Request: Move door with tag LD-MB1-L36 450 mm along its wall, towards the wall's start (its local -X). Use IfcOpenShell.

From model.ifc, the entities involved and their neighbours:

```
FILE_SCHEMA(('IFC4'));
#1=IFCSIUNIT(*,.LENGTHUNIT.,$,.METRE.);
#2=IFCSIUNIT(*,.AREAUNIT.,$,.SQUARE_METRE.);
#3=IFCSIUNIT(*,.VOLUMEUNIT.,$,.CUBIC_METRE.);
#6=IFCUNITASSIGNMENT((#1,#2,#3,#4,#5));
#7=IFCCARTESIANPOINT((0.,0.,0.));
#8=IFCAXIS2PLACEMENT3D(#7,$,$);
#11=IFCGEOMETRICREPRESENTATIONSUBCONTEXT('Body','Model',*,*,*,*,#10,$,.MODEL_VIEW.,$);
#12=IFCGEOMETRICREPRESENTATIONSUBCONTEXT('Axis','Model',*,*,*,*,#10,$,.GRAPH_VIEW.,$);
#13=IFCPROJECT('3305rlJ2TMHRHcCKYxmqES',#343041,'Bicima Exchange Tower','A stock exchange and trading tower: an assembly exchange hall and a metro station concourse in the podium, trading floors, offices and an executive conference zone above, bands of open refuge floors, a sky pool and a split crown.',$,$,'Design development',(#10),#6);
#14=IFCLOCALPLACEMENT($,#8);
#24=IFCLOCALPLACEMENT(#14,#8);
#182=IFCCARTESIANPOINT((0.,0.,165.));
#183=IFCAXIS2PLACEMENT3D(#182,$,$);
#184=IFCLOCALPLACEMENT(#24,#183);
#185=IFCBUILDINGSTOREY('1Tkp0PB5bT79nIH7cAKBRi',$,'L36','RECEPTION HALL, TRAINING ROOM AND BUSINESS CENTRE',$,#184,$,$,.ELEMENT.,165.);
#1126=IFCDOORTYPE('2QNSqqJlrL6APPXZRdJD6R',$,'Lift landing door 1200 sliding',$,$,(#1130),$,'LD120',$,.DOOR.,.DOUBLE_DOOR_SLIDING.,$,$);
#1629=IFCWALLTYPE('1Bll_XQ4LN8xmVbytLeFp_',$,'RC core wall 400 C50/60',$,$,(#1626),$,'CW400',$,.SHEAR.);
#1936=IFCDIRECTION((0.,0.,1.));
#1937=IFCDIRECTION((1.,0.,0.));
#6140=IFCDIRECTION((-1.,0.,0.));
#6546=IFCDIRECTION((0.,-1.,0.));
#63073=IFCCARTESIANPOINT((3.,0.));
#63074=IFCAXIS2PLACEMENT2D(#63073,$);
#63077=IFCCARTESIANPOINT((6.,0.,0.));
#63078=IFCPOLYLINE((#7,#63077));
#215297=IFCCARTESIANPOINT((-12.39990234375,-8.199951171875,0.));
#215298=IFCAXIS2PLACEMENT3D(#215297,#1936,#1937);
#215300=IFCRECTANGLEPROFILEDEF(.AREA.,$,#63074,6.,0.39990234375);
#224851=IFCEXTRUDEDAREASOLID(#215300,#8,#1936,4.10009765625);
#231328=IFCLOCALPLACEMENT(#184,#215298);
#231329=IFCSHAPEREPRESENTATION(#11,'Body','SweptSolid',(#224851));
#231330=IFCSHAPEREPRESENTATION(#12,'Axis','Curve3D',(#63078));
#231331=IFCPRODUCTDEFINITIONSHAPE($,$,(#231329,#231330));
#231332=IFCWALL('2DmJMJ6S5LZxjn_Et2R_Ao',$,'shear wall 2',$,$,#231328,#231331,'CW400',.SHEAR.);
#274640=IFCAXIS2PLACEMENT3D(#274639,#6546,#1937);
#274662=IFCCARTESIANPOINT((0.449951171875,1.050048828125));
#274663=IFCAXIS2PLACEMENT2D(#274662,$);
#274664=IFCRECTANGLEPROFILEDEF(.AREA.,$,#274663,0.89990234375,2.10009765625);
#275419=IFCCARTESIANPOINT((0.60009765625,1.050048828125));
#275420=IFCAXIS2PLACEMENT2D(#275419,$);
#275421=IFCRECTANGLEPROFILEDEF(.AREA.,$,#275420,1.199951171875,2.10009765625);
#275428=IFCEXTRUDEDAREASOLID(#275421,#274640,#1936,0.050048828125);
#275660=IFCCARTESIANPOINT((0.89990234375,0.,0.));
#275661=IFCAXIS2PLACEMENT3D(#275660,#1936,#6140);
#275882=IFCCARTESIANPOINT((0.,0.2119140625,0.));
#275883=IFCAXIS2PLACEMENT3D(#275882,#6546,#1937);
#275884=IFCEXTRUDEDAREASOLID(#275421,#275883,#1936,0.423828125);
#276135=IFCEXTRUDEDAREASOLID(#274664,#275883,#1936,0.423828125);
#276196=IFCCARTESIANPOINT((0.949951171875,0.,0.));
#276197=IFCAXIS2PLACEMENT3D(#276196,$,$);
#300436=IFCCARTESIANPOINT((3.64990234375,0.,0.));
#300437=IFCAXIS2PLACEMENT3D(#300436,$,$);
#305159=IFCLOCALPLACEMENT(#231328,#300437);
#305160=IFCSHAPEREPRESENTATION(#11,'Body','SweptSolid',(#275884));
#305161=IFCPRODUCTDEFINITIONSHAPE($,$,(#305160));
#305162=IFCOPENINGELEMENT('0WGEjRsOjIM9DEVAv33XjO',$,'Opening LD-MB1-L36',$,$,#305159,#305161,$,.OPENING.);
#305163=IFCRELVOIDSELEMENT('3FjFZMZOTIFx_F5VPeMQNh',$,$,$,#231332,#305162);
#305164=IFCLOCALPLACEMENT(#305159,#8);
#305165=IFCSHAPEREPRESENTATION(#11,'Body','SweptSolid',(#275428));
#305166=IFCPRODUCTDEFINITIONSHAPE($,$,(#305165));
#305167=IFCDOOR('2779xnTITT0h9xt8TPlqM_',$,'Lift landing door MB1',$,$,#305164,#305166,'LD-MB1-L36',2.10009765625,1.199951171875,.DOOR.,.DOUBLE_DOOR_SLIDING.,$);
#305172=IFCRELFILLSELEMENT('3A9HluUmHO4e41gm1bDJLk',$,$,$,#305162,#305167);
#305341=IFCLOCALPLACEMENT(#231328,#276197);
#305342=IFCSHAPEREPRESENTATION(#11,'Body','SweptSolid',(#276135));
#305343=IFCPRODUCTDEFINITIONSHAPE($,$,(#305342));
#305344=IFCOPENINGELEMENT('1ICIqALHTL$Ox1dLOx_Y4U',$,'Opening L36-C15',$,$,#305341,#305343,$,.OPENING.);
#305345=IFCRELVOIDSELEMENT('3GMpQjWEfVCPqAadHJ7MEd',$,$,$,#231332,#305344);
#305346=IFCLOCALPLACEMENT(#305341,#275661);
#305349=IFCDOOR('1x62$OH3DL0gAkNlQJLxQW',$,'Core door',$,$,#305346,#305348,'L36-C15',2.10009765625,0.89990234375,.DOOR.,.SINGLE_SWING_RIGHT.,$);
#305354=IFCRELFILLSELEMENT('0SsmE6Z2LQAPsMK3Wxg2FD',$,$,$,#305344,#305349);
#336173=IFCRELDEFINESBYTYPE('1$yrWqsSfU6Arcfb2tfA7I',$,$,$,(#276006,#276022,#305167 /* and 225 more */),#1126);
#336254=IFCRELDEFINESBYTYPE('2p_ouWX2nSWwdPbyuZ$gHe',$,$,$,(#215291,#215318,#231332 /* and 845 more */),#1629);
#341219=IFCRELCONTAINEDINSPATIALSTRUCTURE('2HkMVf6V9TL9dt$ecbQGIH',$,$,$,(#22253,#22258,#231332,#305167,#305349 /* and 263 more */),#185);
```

```python
import ifcopenshell
import ifcopenshell.api.geometry
import ifcopenshell.util.placement
import ifcopenshell.util.unit

model = ifcopenshell.open("model.ifc")
unit_scale = ifcopenshell.util.unit.calculate_unit_scale(model)

door = model.by_guid("2779xnTITT0h9xt8TPlqM_")
opening = door.FillsVoids[0].RelatingOpeningElement
wall = opening.VoidsElements[0].RelatingBuildingElement

wall_matrix = ifcopenshell.util.placement.get_local_placement(wall.ObjectPlacement)
shift = wall_matrix[:3, 0] * -0.45 / unit_scale
before = ifcopenshell.util.placement.get_local_placement(door.ObjectPlacement)[:3, 3].copy()

# The door is placed relative to its opening, so it follows when the opening moves.
matrix = ifcopenshell.util.placement.get_local_placement(opening.ObjectPlacement)
matrix[:3, 3] += shift
ifcopenshell.api.geometry.edit_object_placement(
    model, product=opening, matrix=matrix, is_si=False, should_transform_children=True
)

after = ifcopenshell.util.placement.get_local_placement(door.ObjectPlacement)[:3, 3]
print("door moved by", (after - before).round(3) + 0.0)

model.write("model_v2.ifc")
```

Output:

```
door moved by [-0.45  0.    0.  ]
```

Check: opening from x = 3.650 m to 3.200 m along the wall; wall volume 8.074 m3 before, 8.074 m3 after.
